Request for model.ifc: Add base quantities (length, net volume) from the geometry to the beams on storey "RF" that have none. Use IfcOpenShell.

First a look at what the model holds.

```python
import ifcopenshell
import ifcopenshell.util.element
import ifcopenshell.util.unit

model = ifcopenshell.open("model.ifc")
print(model.schema)
for unit_type in ("LENGTHUNIT", "AREAUNIT", "VOLUMEUNIT"):
    print(unit_type, ifcopenshell.util.unit.calculate_unit_scale(model, unit_type))
storey = next(s for s in model.by_type("IfcBuildingStorey") if s.Name == "RF")
beams = [e for e in ifcopenshell.util.element.get_decomposition(storey) if e.is_a("IfcBeam")]
for e in sorted(beams, key=lambda e: e.id()):
    print(e.id(), e.is_a(), e.Name, list(ifcopenshell.util.element.get_psets(e, qtos_only=True)), sep=" | ")
```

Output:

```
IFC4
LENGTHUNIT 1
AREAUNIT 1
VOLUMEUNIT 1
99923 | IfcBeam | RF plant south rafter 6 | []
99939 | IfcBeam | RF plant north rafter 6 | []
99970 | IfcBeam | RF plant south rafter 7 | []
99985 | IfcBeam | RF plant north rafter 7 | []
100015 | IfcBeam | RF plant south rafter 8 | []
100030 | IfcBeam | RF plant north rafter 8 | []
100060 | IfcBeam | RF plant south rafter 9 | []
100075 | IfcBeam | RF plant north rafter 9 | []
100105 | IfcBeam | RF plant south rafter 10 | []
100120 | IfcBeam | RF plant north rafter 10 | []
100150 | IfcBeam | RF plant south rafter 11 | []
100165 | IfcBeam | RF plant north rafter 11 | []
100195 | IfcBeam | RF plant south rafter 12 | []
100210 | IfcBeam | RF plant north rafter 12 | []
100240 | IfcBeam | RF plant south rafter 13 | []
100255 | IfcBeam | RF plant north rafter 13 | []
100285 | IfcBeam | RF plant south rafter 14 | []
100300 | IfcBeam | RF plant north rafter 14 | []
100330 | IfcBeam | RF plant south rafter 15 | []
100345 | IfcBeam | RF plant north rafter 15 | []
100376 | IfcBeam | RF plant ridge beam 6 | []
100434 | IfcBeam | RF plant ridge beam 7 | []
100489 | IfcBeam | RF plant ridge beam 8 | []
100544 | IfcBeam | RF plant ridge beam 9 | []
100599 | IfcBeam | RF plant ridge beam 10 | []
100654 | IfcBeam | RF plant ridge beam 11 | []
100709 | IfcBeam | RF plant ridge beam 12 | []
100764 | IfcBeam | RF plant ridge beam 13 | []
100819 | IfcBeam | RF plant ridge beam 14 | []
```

```python
import ifcopenshell
import ifcopenshell.api.pset
import ifcopenshell.geom
import ifcopenshell.util.element
import ifcopenshell.util.shape
import ifcopenshell.util.unit

model = ifcopenshell.open("model.ifc")
unit_scale = ifcopenshell.util.unit.calculate_unit_scale(model)
volume_scale = ifcopenshell.util.unit.calculate_unit_scale(model, "VOLUMEUNIT")
settings = ifcopenshell.geom.settings()

storey = next(s for s in model.by_type("IfcBuildingStorey") if s.Name == "RF")
beams = [e for e in ifcopenshell.util.element.get_decomposition(storey) if e.is_a("IfcBeam")]

for e in sorted(beams, key=lambda e: e.id()):
    if ifcopenshell.util.element.get_psets(e, qtos_only=True, should_inherit=False):
        continue
    # Geometry comes back in metres, in the element's own axes.
    shape = ifcopenshell.geom.create_shape(settings, e)
    values = {
        "Length": ifcopenshell.util.shape.get_max_xyz(shape.geometry) / unit_scale,
        "NetVolume": ifcopenshell.util.shape.get_volume(shape.geometry) / volume_scale,
    }
    qto = ifcopenshell.api.pset.add_qto(model, product=e, name="Qto_BeamBaseQuantities")
    ifcopenshell.api.pset.edit_qto(model, qto=qto, properties=values)
    print(e.id(), {k: round(v, 3) for k, v in values.items()})

model.write("model_rev.ifc")
```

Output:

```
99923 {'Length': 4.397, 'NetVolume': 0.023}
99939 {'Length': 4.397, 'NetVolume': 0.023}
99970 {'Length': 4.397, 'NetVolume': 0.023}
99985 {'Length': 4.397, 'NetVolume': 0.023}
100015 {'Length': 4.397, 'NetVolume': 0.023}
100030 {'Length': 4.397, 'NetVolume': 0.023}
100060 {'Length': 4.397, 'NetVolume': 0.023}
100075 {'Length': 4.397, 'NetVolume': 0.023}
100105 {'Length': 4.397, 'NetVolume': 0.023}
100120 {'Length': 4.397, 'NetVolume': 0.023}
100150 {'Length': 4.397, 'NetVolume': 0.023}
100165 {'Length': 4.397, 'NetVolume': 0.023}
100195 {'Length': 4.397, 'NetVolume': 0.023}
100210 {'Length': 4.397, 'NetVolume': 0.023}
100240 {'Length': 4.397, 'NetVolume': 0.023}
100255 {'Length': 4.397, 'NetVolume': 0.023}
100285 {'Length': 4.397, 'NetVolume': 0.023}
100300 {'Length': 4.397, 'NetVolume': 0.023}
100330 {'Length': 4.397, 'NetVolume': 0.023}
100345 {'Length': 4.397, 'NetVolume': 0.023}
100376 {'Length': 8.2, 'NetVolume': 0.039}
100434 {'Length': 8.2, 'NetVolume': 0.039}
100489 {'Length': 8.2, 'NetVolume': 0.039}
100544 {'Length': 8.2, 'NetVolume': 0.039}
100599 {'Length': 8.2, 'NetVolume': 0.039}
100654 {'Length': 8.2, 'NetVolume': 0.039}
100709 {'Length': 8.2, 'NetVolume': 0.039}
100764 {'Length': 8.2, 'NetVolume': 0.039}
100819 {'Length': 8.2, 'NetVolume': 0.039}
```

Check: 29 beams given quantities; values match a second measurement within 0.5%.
